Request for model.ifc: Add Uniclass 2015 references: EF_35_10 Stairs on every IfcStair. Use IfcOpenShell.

First a look at what the model holds.

```python
import ifcopenshell

model = ifcopenshell.open("model.ifc")
print(model.schema)
print("classifications:", [c.Name for c in model.by_type("IfcClassification")])
for ifc_class in ("IfcDoor", "IfcRoof", "IfcStair", "IfcWall", "IfcWindow"):
    print(ifc_class, len(model.by_type(ifc_class)))
```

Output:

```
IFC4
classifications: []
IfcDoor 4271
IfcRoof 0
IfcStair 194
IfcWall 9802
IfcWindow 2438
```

```python
import ifcopenshell
import ifcopenshell.api.classification

model = ifcopenshell.open("model.ifc")

system = ifcopenshell.api.classification.add_classification(model, classification="Uniclass 2015")

codes = {
    "IfcStair": ("EF_35_10", "Stairs"),
}
for ifc_class, (code, name) in codes.items():
    products = model.by_type(ifc_class)
    ifcopenshell.api.classification.add_reference(
        model, products=products, classification=system, identification=code, name=name
    )
    print(code, len(products))

model.write("model-out.ifc")
```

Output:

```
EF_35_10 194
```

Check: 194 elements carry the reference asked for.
